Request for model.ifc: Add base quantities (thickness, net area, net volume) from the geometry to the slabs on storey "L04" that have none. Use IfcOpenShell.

First a look at what the model holds.

```python
import ifcopenshell
import ifcopenshell.util.element
import ifcopenshell.util.unit

model = ifcopenshell.open("model.ifc")
print(model.schema)
for unit_type in ("LENGTHUNIT", "AREAUNIT", "VOLUMEUNIT"):
    print(unit_type, ifcopenshell.util.unit.calculate_unit_scale(model, unit_type))
storey = next(s for s in model.by_type("IfcBuildingStorey") if s.Name == "L04")
slabs = [e for e in ifcopenshell.util.element.get_decomposition(storey) if e.is_a("IfcSlab")]
for e in sorted(slabs, key=lambda e: e.id()):
    print(e.id(), e.is_a(), e.Name, list(ifcopenshell.util.element.get_psets(e, qtos_only=True)), sep=" | ")
```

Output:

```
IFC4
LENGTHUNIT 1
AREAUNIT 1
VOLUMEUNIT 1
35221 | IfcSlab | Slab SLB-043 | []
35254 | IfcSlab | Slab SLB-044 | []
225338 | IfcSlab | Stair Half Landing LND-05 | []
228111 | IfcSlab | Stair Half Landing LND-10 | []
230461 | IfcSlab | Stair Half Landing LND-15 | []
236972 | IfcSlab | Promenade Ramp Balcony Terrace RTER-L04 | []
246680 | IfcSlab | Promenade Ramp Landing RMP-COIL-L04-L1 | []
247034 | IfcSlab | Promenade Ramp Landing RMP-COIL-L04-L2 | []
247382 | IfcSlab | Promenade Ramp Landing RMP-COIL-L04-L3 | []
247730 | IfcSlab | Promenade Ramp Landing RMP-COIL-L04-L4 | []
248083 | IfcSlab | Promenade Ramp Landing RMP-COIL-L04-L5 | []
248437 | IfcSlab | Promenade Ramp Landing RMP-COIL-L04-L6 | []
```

```python
import ifcopenshell
import ifcopenshell.api.pset
import ifcopenshell.geom
import ifcopenshell.util.element
import ifcopenshell.util.shape
import ifcopenshell.util.unit

model = ifcopenshell.open("model.ifc")
unit_scale = ifcopenshell.util.unit.calculate_unit_scale(model)
area_scale = ifcopenshell.util.unit.calculate_unit_scale(model, "AREAUNIT")
volume_scale = ifcopenshell.util.unit.calculate_unit_scale(model, "VOLUMEUNIT")
settings = ifcopenshell.geom.settings()

storey = next(s for s in model.by_type("IfcBuildingStorey") if s.Name == "L04")
slabs = [e for e in ifcopenshell.util.element.get_decomposition(storey) if e.is_a("IfcSlab")]

for e in sorted(slabs, key=lambda e: e.id()):
    if ifcopenshell.util.element.get_psets(e, qtos_only=True, should_inherit=False):
        continue
    # Geometry comes back in metres, in the element's own axes.
    shape = ifcopenshell.geom.create_shape(settings, e)
    values = {
        "Width": ifcopenshell.util.shape.get_z(shape.geometry) / unit_scale,
        "NetArea": ifcopenshell.util.shape.get_footprint_area(shape.geometry) / area_scale,
        "NetVolume": ifcopenshell.util.shape.get_volume(shape.geometry) / volume_scale,
    }
    qto = ifcopenshell.api.pset.add_qto(model, product=e, name="Qto_SlabBaseQuantities")
    ifcopenshell.api.pset.edit_qto(model, qto=qto, properties=values)
    print(e.id(), {k: round(v, 3) for k, v in values.items()})

model.write("model_rev.ifc")
```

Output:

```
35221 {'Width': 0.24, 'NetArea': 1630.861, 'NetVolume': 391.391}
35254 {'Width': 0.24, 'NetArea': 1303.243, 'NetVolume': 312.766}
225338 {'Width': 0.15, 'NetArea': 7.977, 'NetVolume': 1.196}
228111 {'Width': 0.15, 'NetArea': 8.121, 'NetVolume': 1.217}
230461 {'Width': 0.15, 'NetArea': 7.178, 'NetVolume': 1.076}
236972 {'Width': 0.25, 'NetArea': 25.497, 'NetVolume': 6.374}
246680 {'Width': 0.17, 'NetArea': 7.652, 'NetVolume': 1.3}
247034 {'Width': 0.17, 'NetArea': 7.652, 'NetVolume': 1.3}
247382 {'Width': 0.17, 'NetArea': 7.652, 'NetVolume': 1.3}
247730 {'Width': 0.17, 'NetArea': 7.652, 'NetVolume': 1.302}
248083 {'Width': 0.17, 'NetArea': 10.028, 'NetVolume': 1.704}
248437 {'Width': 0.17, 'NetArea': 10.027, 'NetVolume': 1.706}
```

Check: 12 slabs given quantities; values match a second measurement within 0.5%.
